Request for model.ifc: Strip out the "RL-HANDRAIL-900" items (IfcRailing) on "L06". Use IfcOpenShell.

First a look at what the model holds.

```python
import ifcopenshell
import ifcopenshell.util.element

model = ifcopenshell.open("model.ifc")
print(model.schema)
storey = next(s for s in model.by_type("IfcBuildingStorey") if s.Name == "L06")
railings = [e for e in ifcopenshell.util.element.get_decomposition(storey) if e.is_a("IfcRailing")]
seen = {}
for e in railings:
    element_type = ifcopenshell.util.element.get_type(e)
    name = element_type.Name if element_type not in (None, e) else None
    seen[name] = seen.get(name, 0) + 1
for name, count in sorted(seen.items(), key=str):
    print(count, "x", name)
```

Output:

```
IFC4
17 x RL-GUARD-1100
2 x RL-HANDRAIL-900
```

```python
import ifcopenshell
import ifcopenshell.api.root
import ifcopenshell.util.element

model = ifcopenshell.open("model.ifc")

storey = next(s for s in model.by_type("IfcBuildingStorey") if s.Name == "L06")
railings = [e for e in ifcopenshell.util.element.get_decomposition(storey) if e.is_a("IfcRailing")]
targets = [e for e in railings if (t := ifcopenshell.util.element.get_type(e)) not in (None, e) and t.Name == "RL-HANDRAIL-900"]

for e in targets:
    ifcopenshell.api.root.remove_product(model, product=e)
print(len(targets), "removed")

model.write("model_rev.ifc")
```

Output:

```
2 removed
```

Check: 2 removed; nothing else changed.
